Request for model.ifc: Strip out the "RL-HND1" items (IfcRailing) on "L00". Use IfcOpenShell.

First a look at what the model holds.

```python
import ifcopenshell
import ifcopenshell.util.element

model = ifcopenshell.open("model.ifc")
print(model.schema)
storey = next(s for s in model.by_type("IfcBuildingStorey") if s.Name == "L00")
railings = [e for e in ifcopenshell.util.element.get_decomposition(storey) if e.is_a("IfcRailing")]
seen = {}
for e in railings:
    element_type = ifcopenshell.util.element.get_type(e)
    name = element_type.Name if element_type not in (None, e) else None
    seen[name] = seen.get(name, 0) + 1
for name, count in sorted(seen.items(), key=str):
    print(count, "x", name)
```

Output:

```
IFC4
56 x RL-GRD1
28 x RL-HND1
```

```python
import ifcopenshell
import ifcopenshell.api.root
import ifcopenshell.util.element

model = ifcopenshell.open("model.ifc")

storey = next(s for s in model.by_type("IfcBuildingStorey") if s.Name == "L00")
railings = [e for e in ifcopenshell.util.element.get_decomposition(storey) if e.is_a("IfcRailing")]
targets = [e for e in railings if (t := ifcopenshell.util.element.get_type(e)) not in (None, e) and t.Name == "RL-HND1"]

for e in targets:
    ifcopenshell.api.root.remove_product(model, product=e)
print(len(targets), "removed")

model.write("model_rev.ifc")
```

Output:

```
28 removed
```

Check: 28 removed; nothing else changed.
